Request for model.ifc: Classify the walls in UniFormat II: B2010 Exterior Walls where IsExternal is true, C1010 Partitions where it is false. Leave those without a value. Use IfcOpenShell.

First a look at what the model holds.

```python
import ifcopenshell
import ifcopenshell.util.element

model = ifcopenshell.open("model.ifc")
print(model.schema)
print("classifications:", [c.Name for c in model.by_type("IfcClassification")])
values = [ifcopenshell.util.element.get_pset(e, "Pset_WallCommon", "IsExternal") for e in model.by_type("IfcWall")]
for value in (True, False, None):
    print("IsExternal", value, values.count(value))
```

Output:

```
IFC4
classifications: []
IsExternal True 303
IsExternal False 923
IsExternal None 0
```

```python
import ifcopenshell
import ifcopenshell.api.classification
import ifcopenshell.util.element

model = ifcopenshell.open("model.ifc")

system = ifcopenshell.api.classification.add_classification(model, classification="UniFormat II")

walls = model.by_type("IfcWall")
external = {e: ifcopenshell.util.element.get_pset(e, "Pset_WallCommon", "IsExternal") for e in walls}
for flag, code, name in ((True, "B2010", "Exterior Walls"), (False, "C1010", "Partitions")):
    products = [e for e in walls if external[e] is flag]
    ifcopenshell.api.classification.add_reference(
        model, products=products, classification=system, identification=code, name=name
    )
    print(code, len(products))

model.write("model_rev.ifc")
```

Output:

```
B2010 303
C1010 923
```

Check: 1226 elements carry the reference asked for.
